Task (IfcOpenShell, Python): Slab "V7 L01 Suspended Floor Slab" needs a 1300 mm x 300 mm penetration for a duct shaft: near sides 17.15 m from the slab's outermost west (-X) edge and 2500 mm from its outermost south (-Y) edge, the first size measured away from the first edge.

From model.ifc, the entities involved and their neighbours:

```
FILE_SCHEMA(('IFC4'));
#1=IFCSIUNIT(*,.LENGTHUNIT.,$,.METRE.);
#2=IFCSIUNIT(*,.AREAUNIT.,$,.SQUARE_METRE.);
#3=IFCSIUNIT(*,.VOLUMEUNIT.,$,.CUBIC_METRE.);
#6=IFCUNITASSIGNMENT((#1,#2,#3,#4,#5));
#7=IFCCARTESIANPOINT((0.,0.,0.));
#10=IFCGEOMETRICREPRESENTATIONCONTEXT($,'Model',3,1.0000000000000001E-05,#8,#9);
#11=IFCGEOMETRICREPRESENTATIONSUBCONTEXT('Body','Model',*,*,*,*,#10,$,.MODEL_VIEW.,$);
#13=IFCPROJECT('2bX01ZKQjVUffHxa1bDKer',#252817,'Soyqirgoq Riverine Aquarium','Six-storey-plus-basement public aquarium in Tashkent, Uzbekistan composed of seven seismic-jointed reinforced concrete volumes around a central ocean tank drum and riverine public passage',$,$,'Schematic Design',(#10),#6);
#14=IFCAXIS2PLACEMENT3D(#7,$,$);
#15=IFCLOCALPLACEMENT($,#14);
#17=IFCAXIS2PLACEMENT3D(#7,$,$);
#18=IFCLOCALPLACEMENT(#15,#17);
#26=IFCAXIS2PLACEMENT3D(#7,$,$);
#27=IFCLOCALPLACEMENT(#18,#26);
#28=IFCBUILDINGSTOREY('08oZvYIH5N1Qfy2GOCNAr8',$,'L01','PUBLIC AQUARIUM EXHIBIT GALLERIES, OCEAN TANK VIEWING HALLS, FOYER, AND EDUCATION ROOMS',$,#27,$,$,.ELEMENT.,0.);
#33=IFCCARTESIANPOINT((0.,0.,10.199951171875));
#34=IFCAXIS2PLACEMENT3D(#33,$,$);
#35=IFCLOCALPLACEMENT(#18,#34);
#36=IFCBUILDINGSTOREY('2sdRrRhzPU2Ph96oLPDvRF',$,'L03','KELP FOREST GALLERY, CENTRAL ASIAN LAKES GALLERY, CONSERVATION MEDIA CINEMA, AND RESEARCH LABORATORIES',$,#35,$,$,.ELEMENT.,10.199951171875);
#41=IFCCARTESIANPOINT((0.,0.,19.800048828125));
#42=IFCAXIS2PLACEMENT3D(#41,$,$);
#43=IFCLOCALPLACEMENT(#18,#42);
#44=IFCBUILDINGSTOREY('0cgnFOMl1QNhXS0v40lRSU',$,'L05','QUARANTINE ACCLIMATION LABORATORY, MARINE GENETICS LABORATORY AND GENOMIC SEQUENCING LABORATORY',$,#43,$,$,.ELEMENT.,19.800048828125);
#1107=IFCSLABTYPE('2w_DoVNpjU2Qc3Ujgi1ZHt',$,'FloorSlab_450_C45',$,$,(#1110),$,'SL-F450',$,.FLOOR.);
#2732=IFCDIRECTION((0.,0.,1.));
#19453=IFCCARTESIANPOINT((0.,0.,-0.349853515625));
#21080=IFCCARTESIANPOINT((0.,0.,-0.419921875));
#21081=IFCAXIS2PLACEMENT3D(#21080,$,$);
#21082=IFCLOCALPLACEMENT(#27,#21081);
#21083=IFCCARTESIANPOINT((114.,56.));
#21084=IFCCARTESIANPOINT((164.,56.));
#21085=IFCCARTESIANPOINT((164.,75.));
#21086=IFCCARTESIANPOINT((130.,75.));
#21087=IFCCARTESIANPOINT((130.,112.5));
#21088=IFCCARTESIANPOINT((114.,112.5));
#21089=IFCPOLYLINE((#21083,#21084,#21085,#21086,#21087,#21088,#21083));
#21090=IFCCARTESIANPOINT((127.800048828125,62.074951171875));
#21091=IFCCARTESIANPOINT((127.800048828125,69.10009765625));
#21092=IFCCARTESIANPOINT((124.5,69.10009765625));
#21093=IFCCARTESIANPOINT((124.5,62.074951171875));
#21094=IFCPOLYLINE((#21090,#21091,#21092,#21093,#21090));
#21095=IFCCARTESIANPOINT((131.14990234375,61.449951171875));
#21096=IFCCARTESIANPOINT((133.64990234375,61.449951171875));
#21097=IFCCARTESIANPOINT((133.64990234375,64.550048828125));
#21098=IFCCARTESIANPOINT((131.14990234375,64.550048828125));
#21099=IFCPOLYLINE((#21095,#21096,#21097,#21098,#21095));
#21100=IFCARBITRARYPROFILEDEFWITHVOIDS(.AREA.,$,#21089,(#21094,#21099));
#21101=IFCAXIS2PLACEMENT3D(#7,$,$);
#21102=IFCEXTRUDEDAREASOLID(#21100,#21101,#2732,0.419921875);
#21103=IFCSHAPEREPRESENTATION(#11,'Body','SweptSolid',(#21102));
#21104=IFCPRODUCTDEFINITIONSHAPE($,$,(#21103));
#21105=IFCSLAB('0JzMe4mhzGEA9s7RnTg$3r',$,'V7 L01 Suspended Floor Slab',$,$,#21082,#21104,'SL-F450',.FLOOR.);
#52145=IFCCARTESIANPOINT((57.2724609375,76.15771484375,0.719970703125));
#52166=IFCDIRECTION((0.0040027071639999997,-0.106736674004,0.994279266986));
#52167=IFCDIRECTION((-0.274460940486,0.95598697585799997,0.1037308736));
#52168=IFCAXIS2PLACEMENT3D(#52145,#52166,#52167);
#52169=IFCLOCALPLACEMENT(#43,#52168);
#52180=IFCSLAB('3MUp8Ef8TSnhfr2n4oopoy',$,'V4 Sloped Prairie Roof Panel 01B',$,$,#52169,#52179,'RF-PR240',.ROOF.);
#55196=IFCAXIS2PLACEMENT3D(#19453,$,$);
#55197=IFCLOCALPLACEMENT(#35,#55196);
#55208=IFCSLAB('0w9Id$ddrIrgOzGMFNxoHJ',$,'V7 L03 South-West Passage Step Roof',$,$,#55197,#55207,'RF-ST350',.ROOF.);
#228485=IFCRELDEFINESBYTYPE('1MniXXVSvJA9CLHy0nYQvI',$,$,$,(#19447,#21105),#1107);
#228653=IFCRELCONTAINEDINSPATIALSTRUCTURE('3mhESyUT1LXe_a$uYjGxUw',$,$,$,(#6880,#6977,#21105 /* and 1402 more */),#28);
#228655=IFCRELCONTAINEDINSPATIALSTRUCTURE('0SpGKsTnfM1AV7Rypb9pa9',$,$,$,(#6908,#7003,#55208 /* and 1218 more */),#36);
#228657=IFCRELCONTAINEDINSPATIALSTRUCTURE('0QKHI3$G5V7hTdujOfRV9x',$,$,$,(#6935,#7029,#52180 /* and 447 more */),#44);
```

```python
import numpy as np
import ifcopenshell
import ifcopenshell.api.feature
import ifcopenshell.api.geometry
import ifcopenshell.api.root
import ifcopenshell.geom
import ifcopenshell.util.placement
import ifcopenshell.util.representation
import ifcopenshell.util.shape
import ifcopenshell.util.unit

model = ifcopenshell.open("model.ifc")
unit_scale = ifcopenshell.util.unit.calculate_unit_scale(model)
settings = ifcopenshell.geom.settings()


def volume(element):
    """Net volume in cubic metres, openings subtracted."""
    shape = ifcopenshell.geom.create_shape(settings, element)
    return ifcopenshell.util.shape.get_volume(shape.geometry)


slab = model.by_guid("0JzMe4mhzGEA9s7RnTg$3r")
before = volume(slab)

# Extent in the slab's own axes, in metres. The edges named are its -X and -Y sides.
slab_shape = ifcopenshell.geom.create_shape(settings, slab)
vertices = ifcopenshell.util.shape.get_vertices(slab_shape.geometry)
x_min, y_min, bottom = vertices.min(axis=0)
top = vertices[:, 2].max()

opening = ifcopenshell.api.root.create_entity(model, ifc_class="IfcOpeningElement", name="Duct shaft opening", predefined_type="OPENING")
context = ifcopenshell.util.representation.get_context(model, "Model", "Body", "MODEL_VIEW")
width, depth = 1.3, 0.3
outline = [(0.0, 0.0), (width, 0.0), (width, depth), (0.0, depth), (0.0, 0.0)]
# Overshoot both faces by 50 mm so the cut is clean.
shape = ifcopenshell.api.geometry.add_slab_representation(
    model, context=context, depth=top - bottom + 0.1, polyline=outline
)
ifcopenshell.api.geometry.assign_representation(model, product=opening, representation=shape)

matrix = ifcopenshell.util.placement.get_local_placement(slab.ObjectPlacement)
matrix[:, 3] = matrix @ np.append(np.array([x_min + 17.15, y_min + 2.5, bottom - 0.05]) / unit_scale, 1.0)
ifcopenshell.api.geometry.edit_object_placement(model, product=opening, matrix=matrix, is_si=False)
ifcopenshell.api.feature.add_feature(model, feature=opening, element=slab)

after = volume(slab)

print(f"slab volume {before:.3f} -> {after:.3f} m3")

model.write("model_rev.ifc")
```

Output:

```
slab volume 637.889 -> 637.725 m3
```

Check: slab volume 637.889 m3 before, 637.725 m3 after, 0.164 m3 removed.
